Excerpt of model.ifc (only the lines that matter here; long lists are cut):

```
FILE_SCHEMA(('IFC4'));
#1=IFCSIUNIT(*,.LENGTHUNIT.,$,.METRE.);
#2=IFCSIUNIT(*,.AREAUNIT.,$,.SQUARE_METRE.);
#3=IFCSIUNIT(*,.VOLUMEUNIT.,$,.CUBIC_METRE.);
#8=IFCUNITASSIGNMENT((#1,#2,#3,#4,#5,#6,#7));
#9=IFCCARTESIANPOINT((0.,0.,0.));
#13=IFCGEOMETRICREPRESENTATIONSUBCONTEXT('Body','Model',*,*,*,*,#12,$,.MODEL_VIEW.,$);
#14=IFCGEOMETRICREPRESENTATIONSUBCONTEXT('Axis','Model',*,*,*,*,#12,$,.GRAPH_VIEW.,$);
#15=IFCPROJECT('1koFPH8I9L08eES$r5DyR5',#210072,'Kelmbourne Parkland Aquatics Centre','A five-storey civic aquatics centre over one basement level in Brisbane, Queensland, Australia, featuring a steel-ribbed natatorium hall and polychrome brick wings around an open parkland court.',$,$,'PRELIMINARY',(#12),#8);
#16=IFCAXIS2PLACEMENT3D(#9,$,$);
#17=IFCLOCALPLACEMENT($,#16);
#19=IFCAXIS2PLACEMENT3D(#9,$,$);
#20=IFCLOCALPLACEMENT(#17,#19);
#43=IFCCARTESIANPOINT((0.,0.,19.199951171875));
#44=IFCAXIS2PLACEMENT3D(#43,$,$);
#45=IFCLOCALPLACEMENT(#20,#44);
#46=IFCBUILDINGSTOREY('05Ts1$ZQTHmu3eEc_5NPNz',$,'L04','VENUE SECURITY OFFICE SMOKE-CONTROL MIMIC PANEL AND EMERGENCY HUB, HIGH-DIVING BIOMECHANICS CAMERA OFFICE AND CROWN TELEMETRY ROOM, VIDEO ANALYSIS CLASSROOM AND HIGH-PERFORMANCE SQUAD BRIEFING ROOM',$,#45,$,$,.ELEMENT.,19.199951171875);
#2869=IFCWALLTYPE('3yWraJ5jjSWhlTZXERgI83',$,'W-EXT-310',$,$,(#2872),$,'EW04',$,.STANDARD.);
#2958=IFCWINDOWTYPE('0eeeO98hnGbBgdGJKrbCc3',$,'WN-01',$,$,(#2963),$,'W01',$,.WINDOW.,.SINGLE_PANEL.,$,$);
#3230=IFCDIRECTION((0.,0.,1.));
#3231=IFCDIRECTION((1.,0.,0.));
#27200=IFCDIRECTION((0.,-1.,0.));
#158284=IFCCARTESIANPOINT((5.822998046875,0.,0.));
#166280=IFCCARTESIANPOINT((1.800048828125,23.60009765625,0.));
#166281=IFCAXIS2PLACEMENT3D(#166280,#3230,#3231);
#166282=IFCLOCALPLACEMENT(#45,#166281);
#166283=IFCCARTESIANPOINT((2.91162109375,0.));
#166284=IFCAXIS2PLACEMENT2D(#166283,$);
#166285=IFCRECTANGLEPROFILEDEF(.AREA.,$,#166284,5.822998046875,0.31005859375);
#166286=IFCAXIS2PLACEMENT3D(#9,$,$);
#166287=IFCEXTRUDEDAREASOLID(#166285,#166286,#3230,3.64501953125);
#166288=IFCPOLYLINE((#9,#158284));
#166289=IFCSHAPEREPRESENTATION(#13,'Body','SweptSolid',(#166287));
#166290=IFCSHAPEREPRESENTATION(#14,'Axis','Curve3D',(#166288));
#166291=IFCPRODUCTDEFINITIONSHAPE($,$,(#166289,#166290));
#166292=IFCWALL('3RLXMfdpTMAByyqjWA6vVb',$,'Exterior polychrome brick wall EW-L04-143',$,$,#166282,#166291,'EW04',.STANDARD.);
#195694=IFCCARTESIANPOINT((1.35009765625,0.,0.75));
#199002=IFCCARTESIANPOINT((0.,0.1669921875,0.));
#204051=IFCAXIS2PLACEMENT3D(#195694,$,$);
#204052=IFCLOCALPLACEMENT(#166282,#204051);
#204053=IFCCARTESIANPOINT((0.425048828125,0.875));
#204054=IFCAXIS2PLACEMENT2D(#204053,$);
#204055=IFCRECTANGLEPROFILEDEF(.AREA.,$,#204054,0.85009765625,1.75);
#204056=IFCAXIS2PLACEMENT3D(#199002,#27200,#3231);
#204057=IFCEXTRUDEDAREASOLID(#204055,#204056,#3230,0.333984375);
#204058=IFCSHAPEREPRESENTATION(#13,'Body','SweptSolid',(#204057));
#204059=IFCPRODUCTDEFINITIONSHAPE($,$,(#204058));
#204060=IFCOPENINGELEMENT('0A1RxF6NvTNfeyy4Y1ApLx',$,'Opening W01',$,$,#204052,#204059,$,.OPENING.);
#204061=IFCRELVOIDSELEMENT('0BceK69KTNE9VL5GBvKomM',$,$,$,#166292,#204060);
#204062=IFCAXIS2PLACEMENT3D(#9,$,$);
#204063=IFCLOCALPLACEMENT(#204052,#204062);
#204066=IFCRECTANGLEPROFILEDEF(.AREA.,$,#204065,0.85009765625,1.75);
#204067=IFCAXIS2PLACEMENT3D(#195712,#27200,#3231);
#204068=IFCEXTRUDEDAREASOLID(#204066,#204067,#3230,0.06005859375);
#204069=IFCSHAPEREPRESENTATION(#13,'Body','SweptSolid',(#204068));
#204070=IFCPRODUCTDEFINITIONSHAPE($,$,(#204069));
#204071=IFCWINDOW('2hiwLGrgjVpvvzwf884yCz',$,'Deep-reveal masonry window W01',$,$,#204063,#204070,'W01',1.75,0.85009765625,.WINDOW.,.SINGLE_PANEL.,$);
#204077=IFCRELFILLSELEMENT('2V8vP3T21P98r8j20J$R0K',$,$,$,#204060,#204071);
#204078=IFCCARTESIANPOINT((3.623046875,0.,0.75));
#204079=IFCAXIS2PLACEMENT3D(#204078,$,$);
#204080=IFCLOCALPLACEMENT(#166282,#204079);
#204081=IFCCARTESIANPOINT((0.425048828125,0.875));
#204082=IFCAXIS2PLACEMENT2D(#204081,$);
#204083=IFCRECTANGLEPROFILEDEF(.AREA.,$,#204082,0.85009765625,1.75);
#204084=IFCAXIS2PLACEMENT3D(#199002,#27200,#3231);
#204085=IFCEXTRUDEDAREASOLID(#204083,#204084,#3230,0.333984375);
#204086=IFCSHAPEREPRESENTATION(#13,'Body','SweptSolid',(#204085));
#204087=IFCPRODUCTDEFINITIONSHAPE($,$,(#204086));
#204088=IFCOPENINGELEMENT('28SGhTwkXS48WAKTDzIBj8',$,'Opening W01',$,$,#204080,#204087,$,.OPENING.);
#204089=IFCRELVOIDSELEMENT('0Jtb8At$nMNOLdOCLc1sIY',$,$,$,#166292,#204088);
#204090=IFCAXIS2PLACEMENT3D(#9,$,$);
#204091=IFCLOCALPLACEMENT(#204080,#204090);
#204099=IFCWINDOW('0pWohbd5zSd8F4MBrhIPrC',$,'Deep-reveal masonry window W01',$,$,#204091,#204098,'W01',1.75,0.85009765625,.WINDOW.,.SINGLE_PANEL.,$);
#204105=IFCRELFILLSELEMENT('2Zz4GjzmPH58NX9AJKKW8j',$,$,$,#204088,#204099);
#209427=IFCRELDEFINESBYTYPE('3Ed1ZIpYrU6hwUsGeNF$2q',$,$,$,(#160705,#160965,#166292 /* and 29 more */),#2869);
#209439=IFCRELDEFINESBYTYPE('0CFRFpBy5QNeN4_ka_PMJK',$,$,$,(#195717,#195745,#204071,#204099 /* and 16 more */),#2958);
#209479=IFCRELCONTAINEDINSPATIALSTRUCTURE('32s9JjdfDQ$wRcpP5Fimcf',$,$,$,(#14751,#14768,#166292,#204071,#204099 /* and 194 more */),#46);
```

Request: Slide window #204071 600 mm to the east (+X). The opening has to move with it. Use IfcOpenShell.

```python
import ifcopenshell
import ifcopenshell.api.geometry
import ifcopenshell.util.placement
import ifcopenshell.util.unit

model = ifcopenshell.open("model.ifc")
unit_scale = ifcopenshell.util.unit.calculate_unit_scale(model)

window = model.by_guid("2hiwLGrgjVpvvzwf884yCz")
opening = window.FillsVoids[0].RelatingOpeningElement
wall = opening.VoidsElements[0].RelatingBuildingElement

wall_matrix = ifcopenshell.util.placement.get_local_placement(wall.ObjectPlacement)
shift = wall_matrix[:3, 0] * 0.6 / unit_scale
before = ifcopenshell.util.placement.get_local_placement(window.ObjectPlacement)[:3, 3].copy()

# The window is placed relative to its opening, so it follows when the opening moves.
matrix = ifcopenshell.util.placement.get_local_placement(opening.ObjectPlacement)
matrix[:3, 3] += shift
ifcopenshell.api.geometry.edit_object_placement(
    model, product=opening, matrix=matrix, is_si=False, should_transform_children=True
)

after = ifcopenshell.util.placement.get_local_placement(window.ObjectPlacement)[:3, 3]
print("window moved by", (after - before).round(3) + 0.0)

model.write("model_v2.ifc")
```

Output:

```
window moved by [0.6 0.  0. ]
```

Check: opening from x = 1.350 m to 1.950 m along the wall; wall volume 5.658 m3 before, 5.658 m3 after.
